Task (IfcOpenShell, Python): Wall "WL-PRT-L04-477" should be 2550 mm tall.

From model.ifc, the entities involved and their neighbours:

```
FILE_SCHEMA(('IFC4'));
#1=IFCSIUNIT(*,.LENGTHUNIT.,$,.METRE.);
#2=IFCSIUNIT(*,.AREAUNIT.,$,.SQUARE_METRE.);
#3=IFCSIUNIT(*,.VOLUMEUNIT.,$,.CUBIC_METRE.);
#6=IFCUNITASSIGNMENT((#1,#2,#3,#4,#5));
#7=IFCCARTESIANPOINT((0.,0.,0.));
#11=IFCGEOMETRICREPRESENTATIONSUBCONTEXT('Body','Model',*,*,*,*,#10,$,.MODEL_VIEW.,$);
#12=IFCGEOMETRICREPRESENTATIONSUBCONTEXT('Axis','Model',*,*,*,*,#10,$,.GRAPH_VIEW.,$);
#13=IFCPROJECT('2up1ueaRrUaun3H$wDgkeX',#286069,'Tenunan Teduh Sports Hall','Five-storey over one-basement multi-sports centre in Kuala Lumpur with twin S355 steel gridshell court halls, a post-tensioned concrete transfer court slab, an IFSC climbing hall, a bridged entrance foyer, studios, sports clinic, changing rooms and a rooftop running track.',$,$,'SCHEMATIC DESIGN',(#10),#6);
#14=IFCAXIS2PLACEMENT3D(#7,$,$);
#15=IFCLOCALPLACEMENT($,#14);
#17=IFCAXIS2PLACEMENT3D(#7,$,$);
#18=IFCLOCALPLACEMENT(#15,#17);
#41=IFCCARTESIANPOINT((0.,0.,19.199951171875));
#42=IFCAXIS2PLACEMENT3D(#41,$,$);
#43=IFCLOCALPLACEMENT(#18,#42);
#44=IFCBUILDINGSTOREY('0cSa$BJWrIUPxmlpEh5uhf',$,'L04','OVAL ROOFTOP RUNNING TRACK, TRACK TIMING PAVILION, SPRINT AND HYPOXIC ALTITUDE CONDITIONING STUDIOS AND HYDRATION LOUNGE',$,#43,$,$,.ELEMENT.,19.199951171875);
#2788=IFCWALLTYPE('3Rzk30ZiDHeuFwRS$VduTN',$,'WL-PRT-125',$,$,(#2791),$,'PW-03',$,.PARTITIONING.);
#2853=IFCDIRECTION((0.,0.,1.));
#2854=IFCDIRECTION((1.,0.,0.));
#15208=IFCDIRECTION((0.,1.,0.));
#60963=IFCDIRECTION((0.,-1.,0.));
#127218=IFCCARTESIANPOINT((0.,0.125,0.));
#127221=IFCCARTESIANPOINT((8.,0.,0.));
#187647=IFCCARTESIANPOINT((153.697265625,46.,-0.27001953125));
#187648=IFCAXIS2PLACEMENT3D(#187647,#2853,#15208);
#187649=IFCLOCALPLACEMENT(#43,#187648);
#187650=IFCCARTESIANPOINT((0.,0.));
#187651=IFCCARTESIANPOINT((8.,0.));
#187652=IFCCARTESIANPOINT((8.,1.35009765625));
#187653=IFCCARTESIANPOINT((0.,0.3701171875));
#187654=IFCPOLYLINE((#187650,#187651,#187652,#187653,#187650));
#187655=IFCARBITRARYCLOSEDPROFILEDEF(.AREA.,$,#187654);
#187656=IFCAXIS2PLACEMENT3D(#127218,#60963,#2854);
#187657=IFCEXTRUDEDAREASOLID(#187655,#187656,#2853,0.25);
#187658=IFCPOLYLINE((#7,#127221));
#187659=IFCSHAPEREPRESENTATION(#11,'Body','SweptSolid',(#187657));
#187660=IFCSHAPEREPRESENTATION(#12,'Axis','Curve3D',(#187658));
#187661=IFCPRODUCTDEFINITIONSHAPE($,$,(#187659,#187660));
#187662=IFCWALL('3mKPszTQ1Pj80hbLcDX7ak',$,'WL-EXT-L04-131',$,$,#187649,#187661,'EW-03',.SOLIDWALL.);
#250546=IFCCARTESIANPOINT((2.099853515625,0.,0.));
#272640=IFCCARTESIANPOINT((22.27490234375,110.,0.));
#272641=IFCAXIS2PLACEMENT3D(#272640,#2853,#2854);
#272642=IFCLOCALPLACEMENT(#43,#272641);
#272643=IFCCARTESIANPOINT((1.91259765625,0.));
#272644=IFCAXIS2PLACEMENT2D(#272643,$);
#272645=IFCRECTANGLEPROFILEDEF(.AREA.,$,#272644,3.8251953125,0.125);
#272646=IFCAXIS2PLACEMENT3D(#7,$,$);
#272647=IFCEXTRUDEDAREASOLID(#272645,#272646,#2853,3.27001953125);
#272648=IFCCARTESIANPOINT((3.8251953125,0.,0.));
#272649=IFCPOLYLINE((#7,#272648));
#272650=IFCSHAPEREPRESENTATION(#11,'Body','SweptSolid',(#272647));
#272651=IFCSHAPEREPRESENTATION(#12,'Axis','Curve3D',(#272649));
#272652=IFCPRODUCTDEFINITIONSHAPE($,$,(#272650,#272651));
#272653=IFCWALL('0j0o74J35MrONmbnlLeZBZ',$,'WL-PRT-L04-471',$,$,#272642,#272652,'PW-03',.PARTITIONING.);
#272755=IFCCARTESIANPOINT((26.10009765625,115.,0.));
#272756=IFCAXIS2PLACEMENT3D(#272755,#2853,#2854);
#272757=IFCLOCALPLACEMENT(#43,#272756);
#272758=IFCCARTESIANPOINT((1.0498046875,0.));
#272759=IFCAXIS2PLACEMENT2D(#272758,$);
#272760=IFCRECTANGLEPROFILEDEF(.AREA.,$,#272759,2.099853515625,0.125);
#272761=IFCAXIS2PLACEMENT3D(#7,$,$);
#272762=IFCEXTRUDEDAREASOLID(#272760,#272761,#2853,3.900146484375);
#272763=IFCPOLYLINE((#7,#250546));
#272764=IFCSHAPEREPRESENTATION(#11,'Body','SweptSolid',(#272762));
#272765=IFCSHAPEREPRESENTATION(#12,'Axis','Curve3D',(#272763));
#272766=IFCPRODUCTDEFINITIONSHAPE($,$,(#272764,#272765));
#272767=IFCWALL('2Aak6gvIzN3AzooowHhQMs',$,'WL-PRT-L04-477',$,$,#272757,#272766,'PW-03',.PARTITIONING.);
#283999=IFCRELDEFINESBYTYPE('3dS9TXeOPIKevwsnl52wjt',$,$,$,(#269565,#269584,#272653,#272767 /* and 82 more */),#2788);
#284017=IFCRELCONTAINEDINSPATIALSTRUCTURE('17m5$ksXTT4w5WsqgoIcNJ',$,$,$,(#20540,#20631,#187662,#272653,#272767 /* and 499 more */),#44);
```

```python
import ifcopenshell
import ifcopenshell.geom
import ifcopenshell.util.representation
import ifcopenshell.util.shape
import ifcopenshell.util.unit

model = ifcopenshell.open("model.ifc")
unit_scale = ifcopenshell.util.unit.calculate_unit_scale(model)
settings = ifcopenshell.geom.settings()


def volume(element):
    """Net volume in cubic metres, openings subtracted."""
    shape = ifcopenshell.geom.create_shape(settings, element)
    return ifcopenshell.util.shape.get_volume(shape.geometry)


wall = model.by_id(272767)
before = volume(wall)

body = ifcopenshell.util.representation.get_representation(wall, "Model", "Body")
solid = body.Items[0]
old_height = solid.Depth
solid.Depth = 2.55 / unit_scale
after = volume(wall)

print(f"height {old_height:g} -> {solid.Depth:g}, volume {before:.3f} -> {after:.3f} m3")

model.write("model-out.ifc")
```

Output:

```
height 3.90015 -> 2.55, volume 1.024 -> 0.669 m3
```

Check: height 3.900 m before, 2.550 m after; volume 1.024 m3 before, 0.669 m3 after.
